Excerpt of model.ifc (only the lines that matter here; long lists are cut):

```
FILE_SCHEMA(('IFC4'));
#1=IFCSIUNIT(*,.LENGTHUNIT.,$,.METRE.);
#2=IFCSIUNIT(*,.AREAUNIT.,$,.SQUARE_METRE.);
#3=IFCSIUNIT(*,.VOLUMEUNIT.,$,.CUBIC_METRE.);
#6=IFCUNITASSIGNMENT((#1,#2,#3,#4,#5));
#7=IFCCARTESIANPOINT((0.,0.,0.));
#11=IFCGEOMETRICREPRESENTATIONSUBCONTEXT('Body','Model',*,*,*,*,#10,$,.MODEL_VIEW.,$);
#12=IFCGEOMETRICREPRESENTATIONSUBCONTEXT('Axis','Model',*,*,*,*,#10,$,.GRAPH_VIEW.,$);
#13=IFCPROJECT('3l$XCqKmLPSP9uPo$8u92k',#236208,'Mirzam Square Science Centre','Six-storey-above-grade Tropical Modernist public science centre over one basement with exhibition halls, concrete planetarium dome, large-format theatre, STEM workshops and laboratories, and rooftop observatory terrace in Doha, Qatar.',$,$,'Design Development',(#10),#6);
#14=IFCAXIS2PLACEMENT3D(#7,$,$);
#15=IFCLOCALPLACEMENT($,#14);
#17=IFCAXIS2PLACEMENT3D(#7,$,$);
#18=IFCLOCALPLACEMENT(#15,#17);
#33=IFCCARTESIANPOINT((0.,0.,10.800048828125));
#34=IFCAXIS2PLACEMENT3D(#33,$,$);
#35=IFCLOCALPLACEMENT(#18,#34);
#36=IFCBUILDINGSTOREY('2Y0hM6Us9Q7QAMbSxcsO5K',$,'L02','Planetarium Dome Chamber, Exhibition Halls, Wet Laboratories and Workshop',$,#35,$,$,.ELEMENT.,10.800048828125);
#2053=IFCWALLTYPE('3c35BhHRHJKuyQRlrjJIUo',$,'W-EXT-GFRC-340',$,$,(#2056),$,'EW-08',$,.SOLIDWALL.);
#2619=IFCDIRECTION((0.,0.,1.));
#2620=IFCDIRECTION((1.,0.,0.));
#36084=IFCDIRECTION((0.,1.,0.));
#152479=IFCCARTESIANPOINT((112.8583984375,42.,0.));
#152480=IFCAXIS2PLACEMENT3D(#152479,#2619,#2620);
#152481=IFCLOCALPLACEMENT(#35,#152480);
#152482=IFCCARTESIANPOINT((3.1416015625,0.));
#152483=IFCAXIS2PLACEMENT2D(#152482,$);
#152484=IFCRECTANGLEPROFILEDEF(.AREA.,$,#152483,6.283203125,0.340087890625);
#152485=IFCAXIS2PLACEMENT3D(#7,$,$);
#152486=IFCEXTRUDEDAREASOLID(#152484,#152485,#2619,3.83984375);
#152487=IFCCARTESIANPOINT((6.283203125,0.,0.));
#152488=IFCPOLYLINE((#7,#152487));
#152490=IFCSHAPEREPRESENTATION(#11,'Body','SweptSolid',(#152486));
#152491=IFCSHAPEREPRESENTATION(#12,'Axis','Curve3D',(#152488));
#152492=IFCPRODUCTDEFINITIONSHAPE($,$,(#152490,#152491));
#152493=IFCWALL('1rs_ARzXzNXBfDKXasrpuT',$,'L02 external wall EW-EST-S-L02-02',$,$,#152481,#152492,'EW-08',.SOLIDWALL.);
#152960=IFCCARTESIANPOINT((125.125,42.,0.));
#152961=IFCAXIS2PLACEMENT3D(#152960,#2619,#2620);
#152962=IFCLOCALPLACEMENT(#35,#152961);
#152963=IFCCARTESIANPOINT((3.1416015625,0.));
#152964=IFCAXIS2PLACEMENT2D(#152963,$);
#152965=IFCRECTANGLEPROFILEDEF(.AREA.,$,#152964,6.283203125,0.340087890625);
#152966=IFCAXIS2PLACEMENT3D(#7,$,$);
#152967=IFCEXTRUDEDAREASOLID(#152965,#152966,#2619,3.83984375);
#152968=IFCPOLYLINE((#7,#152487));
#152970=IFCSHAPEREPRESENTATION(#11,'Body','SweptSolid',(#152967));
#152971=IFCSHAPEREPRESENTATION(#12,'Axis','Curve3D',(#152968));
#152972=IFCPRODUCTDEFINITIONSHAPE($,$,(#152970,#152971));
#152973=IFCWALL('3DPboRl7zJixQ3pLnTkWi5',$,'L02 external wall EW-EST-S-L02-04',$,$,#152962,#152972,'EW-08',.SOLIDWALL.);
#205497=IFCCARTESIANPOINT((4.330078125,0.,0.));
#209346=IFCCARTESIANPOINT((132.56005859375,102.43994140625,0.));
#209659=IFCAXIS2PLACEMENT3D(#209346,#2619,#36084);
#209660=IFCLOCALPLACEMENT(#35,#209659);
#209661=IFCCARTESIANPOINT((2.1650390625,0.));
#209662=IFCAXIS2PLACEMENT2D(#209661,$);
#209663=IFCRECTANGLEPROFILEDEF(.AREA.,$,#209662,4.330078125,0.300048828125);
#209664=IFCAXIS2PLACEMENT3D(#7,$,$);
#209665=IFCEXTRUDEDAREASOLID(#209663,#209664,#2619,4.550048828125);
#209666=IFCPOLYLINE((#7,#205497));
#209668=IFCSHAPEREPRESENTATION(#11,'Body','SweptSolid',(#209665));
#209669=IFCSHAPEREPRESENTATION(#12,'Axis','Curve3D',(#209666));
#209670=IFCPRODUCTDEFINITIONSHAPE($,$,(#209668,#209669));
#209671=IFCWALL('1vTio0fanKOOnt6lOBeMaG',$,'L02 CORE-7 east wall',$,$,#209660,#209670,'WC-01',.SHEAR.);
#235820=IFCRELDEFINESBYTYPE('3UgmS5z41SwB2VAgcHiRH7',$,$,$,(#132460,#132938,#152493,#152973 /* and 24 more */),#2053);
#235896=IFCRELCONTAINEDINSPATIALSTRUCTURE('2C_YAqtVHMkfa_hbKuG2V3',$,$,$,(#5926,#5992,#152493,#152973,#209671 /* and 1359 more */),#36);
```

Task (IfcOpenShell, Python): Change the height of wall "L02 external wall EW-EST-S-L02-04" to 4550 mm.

```python
import ifcopenshell
import ifcopenshell.geom
import ifcopenshell.util.representation
import ifcopenshell.util.shape
import ifcopenshell.util.unit

model = ifcopenshell.open("model.ifc")
unit_scale = ifcopenshell.util.unit.calculate_unit_scale(model)
settings = ifcopenshell.geom.settings()


def volume(element):
    """Net volume in cubic metres, openings subtracted."""
    shape = ifcopenshell.geom.create_shape(settings, element)
    return ifcopenshell.util.shape.get_volume(shape.geometry)


wall = model.by_guid("3DPboRl7zJixQ3pLnTkWi5")
before = volume(wall)

body = ifcopenshell.util.representation.get_representation(wall, "Model", "Body")
solid = body.Items[0]
old_height = solid.Depth
solid.Depth = 4.55 / unit_scale
after = volume(wall)

print(f"height {old_height:g} -> {solid.Depth:g}, volume {before:.3f} -> {after:.3f} m3")

model.write("model_edited.ifc")
```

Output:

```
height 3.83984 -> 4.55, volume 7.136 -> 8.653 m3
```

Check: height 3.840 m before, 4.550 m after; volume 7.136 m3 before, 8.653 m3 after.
